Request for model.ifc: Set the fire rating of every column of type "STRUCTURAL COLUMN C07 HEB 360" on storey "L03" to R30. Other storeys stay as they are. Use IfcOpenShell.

First a look at what the model holds.

```python
import ifcopenshell
import ifcopenshell.util.element

model = ifcopenshell.open("model.ifc")
print(model.schema)
storey = next(s for s in model.by_type("IfcBuildingStorey") if s.Name == "L03")
columns = [e for e in ifcopenshell.util.element.get_decomposition(storey) if e.is_a("IfcColumn")]
seen = {}
for e in columns:
    element_type = ifcopenshell.util.element.get_type(e)
    key = (element_type.Name if element_type != e and element_type else None, ifcopenshell.util.element.get_pset(e, "Pset_ColumnCommon", "FireRating"))
    seen[key] = seen.get(key, 0) + 1
for (name, value), count in sorted(seen.items(), key=str):
    print(count, "x", name, "|", value)
```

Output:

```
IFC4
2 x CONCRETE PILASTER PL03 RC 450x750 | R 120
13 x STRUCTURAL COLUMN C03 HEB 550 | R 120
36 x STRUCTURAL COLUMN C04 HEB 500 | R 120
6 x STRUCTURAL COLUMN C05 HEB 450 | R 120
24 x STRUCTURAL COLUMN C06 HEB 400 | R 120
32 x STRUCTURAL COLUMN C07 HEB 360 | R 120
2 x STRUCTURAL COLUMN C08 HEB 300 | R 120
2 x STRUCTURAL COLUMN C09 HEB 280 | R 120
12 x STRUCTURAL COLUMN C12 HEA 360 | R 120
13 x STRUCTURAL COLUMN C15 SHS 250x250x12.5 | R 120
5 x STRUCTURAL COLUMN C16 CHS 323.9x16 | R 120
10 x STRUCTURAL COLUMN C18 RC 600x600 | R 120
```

```python
import ifcopenshell
import ifcopenshell.api.pset
import ifcopenshell.util.element

model = ifcopenshell.open("model.ifc")

storey = next(s for s in model.by_type("IfcBuildingStorey") if s.Name == "L03")
columns = [e for e in ifcopenshell.util.element.get_decomposition(storey) if e.is_a("IfcColumn")]

count = 0
for e in columns:
    element_type = ifcopenshell.util.element.get_type(e)
    if element_type in (None, e) or element_type.Name != "STRUCTURAL COLUMN C07 HEB 360":
        continue
    # add_pset returns the element's existing set when there is one.
    pset = ifcopenshell.api.pset.add_pset(model, product=e, name="Pset_ColumnCommon")
    ifcopenshell.api.pset.edit_pset(model, pset=pset, properties={"FireRating": "R30"})
    count += 1

print(count, "columns updated")

model.write("model-out.ifc")
```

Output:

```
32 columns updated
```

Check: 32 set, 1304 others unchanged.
